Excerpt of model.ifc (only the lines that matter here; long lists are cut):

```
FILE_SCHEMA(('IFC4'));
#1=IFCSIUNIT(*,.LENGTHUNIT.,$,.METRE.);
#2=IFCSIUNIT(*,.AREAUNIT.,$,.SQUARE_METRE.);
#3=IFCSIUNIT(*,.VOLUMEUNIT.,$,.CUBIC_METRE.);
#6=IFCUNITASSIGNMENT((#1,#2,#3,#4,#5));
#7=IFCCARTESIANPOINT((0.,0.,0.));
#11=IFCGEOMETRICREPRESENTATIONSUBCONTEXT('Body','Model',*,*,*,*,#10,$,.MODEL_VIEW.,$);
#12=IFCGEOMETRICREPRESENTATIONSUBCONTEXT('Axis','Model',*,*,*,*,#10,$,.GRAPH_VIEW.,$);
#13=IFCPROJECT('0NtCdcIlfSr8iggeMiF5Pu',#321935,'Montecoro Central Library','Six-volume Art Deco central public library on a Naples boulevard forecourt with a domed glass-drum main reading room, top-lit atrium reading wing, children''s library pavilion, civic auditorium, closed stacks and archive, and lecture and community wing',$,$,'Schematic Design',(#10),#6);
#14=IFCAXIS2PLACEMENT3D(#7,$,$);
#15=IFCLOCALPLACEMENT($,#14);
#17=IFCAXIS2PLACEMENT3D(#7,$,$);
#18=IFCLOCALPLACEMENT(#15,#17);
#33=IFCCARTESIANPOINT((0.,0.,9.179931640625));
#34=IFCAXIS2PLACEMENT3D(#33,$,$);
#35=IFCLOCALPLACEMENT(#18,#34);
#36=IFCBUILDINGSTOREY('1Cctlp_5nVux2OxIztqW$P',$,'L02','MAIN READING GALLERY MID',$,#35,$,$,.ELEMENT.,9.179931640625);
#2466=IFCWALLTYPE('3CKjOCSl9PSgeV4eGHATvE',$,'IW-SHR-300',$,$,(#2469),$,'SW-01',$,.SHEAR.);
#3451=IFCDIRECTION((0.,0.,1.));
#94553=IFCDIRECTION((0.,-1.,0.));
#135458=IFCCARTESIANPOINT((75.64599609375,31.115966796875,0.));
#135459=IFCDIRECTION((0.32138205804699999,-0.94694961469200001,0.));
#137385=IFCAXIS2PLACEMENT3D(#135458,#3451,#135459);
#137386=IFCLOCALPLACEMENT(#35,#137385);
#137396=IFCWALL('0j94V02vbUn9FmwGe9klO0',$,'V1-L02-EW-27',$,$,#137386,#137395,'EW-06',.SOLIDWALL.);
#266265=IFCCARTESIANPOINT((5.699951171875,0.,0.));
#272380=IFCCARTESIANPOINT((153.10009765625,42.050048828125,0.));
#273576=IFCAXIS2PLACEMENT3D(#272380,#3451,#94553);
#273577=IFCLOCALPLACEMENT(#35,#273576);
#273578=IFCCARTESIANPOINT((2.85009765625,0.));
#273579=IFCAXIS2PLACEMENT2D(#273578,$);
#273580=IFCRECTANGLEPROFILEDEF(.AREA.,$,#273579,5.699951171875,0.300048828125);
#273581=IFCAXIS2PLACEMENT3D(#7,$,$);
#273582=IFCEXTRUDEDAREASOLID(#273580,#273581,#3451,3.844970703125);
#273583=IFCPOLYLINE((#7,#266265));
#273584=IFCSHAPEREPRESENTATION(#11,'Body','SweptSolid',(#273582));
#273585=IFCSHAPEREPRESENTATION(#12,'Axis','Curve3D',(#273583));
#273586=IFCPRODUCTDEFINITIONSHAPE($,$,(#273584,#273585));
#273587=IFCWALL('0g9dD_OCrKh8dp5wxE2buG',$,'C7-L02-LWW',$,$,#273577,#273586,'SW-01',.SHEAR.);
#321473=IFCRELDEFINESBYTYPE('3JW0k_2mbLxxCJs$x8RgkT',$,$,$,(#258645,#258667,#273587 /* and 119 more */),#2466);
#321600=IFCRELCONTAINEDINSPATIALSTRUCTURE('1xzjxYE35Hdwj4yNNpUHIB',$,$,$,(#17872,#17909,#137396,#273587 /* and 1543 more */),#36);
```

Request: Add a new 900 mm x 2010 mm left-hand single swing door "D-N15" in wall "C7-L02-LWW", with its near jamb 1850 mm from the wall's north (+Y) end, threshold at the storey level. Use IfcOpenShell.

```python
import numpy as np
import ifcopenshell
import ifcopenshell.api.feature
import ifcopenshell.api.geometry
import ifcopenshell.api.root
import ifcopenshell.api.spatial
import ifcopenshell.geom
import ifcopenshell.util.element
import ifcopenshell.util.placement
import ifcopenshell.util.representation
import ifcopenshell.util.shape
import ifcopenshell.util.unit

model = ifcopenshell.open("model.ifc")
unit_scale = ifcopenshell.util.unit.calculate_unit_scale(model)
settings = ifcopenshell.geom.settings()


def volume(element):
    """Net volume in cubic metres, openings subtracted."""
    shape = ifcopenshell.geom.create_shape(settings, element)
    return ifcopenshell.util.shape.get_volume(shape.geometry)


wall = model.by_guid("0g9dD_OCrKh8dp5wxE2buG")
storey = ifcopenshell.util.element.get_container(wall, ifc_class="IfcBuildingStorey")
context = ifcopenshell.util.representation.get_context(model, "Model", "Body", "MODEL_VIEW")
before = volume(wall)

width, height, from_end, sill = 0.9, 2.01, 1.85, 0.0  # metres

# The wall runs along its own X axis, and the end named is its -X end.
wall_shape = ifcopenshell.geom.create_shape(settings, wall)
x, y, z = ifcopenshell.util.shape.get_vertices(wall_shape.geometry).T
start = x.min() + from_end
face, thickness = float(y.min()), float(y.max() - y.min())
wall_matrix = ifcopenshell.util.placement.get_local_placement(wall.ObjectPlacement)
level = ifcopenshell.util.placement.get_local_placement(storey.ObjectPlacement)[2, 3]


def in_wall(x, y):
    """Placement at x, y metres in the wall's axes, at sill height."""
    matrix = wall_matrix.copy()
    matrix[:, 3] = wall_matrix @ np.array([x / unit_scale, y / unit_scale, 0.0, 1.0])
    matrix[2, 3] = level + sill / unit_scale
    return matrix


# Opening: a box that overshoots both wall faces by 50 mm.
opening = ifcopenshell.api.root.create_entity(model, ifc_class="IfcOpeningElement", predefined_type="OPENING")
box = ifcopenshell.api.geometry.add_wall_representation(
    model, context=context, length=width, height=height, thickness=thickness + 0.1
)
ifcopenshell.api.geometry.assign_representation(model, product=opening, representation=box)
ifcopenshell.api.geometry.edit_object_placement(model, product=opening, matrix=in_wall(start, face - 0.05), is_si=False)
ifcopenshell.api.feature.add_feature(model, feature=opening, element=wall)

door = ifcopenshell.api.root.create_entity(model, ifc_class="IfcDoor", name="D-N15", predefined_type="DOOR")
door.OverallWidth, door.OverallHeight = width / unit_scale, height / unit_scale
door.OperationType = "SINGLE_SWING_LEFT"
body = ifcopenshell.api.geometry.add_door_representation(
    model,
    context=context,
    overall_width=door.OverallWidth,
    overall_height=door.OverallHeight,
    operation_type="SINGLE_SWING_LEFT",
    lining_properties={"LiningDepth": thickness / unit_scale, "ThresholdDepth": thickness / unit_scale},
)
ifcopenshell.api.geometry.assign_representation(model, product=door, representation=body)
ifcopenshell.api.spatial.assign_container(model, products=[door], relating_structure=storey)
ifcopenshell.api.feature.add_filling(model, opening=opening, element=door)

# The lining spans the wall, so the door starts at the wall face.
ifcopenshell.api.geometry.edit_object_placement(model, product=door, matrix=in_wall(start, face), is_si=False)

after = volume(wall)

print(f"wall volume {before:.3f} -> {after:.3f} m3")

model.write("model_v2.ifc")
```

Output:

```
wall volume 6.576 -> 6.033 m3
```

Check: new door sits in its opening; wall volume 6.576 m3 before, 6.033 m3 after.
